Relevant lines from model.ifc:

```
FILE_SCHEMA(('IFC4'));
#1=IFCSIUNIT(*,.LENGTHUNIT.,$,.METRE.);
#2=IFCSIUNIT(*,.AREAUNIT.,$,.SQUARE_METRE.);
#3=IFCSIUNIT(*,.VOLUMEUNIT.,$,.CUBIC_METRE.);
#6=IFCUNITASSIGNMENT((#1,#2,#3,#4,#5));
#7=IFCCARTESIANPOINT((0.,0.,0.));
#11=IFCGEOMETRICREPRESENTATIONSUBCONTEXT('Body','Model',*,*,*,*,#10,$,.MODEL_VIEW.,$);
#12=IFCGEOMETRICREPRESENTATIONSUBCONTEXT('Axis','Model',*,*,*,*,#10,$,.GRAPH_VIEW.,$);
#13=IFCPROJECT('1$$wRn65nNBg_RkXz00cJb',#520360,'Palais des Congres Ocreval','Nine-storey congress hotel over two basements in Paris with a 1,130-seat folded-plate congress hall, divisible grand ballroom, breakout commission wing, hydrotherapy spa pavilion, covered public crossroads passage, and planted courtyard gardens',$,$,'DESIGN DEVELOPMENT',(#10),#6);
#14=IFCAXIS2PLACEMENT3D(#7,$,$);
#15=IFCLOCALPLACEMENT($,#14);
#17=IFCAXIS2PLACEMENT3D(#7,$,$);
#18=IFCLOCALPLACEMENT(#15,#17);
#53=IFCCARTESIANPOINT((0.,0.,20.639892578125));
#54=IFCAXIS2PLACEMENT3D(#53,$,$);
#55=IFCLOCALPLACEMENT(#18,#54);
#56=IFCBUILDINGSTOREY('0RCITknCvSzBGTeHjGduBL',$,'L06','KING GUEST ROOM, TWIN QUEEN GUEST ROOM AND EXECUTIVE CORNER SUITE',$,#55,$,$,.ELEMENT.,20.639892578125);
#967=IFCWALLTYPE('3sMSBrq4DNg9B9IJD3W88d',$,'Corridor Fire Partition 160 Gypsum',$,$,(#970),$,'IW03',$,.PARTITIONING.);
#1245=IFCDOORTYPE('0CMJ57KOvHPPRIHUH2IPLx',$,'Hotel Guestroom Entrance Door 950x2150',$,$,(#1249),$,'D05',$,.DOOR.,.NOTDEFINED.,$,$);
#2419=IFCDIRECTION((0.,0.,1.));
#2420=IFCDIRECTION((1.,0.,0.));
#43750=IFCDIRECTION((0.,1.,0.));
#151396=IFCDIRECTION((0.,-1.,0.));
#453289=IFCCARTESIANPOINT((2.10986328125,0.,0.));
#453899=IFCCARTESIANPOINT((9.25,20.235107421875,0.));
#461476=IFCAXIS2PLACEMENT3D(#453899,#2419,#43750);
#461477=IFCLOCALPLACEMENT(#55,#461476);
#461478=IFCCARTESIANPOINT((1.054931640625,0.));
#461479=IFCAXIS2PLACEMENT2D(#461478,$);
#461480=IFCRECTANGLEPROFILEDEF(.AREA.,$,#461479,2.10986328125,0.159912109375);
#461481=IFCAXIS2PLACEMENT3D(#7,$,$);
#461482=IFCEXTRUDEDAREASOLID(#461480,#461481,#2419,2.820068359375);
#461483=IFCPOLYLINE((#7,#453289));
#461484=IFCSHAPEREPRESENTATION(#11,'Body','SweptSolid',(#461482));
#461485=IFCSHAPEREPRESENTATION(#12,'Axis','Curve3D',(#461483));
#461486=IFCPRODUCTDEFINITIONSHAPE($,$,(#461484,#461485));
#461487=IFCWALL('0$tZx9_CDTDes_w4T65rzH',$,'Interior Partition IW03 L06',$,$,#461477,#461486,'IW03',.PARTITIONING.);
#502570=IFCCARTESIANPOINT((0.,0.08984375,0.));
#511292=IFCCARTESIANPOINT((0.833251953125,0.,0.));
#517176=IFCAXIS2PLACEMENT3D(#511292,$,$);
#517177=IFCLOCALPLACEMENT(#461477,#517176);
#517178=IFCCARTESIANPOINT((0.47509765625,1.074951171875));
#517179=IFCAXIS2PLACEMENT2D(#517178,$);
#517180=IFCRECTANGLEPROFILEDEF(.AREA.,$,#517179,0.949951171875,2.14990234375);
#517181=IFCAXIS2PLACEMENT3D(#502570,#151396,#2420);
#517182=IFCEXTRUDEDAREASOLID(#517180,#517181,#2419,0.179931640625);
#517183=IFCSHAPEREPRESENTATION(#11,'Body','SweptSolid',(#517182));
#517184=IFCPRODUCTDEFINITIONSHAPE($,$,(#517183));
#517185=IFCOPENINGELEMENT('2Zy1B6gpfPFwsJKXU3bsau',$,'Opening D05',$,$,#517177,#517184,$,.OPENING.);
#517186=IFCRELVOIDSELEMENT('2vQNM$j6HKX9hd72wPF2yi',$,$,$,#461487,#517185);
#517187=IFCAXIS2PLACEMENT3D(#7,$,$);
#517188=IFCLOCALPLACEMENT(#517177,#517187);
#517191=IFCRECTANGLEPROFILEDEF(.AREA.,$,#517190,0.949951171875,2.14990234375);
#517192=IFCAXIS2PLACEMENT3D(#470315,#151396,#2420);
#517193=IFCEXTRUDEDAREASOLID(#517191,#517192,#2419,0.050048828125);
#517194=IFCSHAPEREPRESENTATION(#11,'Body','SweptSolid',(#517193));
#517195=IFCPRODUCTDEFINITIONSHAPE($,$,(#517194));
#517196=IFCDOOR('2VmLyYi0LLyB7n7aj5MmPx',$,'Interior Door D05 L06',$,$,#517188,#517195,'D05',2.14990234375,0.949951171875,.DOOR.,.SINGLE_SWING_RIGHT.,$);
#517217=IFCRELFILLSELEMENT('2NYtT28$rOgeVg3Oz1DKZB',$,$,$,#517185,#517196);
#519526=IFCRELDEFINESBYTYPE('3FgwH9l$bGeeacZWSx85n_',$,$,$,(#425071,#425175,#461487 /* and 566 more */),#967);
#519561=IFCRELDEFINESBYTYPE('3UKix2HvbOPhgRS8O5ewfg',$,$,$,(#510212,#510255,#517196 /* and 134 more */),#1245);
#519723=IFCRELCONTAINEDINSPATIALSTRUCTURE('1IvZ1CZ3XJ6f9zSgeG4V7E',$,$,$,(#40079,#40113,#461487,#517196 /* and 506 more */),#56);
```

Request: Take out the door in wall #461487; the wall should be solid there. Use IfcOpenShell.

```python
import ifcopenshell
import ifcopenshell.api.feature
import ifcopenshell.api.root
import ifcopenshell.geom
import ifcopenshell.util.shape

model = ifcopenshell.open("model.ifc")
settings = ifcopenshell.geom.settings()


def volume(element):
    """Net volume in cubic metres, openings subtracted."""
    shape = ifcopenshell.geom.create_shape(settings, element)
    return ifcopenshell.util.shape.get_volume(shape.geometry)


door = model.by_guid("2VmLyYi0LLyB7n7aj5MmPx")
opening = door.FillsVoids[0].RelatingOpeningElement
wall = opening.VoidsElements[0].RelatingBuildingElement
before = volume(wall)

ifcopenshell.api.root.remove_product(model, product=door)
ifcopenshell.api.feature.remove_feature(model, feature=opening)

after = volume(wall)

print(f"wall volume {before:.3f} -> {after:.3f} m3")

model.write("model_rev.ifc")
```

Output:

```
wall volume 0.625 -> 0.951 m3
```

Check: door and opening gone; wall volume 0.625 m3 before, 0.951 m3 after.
